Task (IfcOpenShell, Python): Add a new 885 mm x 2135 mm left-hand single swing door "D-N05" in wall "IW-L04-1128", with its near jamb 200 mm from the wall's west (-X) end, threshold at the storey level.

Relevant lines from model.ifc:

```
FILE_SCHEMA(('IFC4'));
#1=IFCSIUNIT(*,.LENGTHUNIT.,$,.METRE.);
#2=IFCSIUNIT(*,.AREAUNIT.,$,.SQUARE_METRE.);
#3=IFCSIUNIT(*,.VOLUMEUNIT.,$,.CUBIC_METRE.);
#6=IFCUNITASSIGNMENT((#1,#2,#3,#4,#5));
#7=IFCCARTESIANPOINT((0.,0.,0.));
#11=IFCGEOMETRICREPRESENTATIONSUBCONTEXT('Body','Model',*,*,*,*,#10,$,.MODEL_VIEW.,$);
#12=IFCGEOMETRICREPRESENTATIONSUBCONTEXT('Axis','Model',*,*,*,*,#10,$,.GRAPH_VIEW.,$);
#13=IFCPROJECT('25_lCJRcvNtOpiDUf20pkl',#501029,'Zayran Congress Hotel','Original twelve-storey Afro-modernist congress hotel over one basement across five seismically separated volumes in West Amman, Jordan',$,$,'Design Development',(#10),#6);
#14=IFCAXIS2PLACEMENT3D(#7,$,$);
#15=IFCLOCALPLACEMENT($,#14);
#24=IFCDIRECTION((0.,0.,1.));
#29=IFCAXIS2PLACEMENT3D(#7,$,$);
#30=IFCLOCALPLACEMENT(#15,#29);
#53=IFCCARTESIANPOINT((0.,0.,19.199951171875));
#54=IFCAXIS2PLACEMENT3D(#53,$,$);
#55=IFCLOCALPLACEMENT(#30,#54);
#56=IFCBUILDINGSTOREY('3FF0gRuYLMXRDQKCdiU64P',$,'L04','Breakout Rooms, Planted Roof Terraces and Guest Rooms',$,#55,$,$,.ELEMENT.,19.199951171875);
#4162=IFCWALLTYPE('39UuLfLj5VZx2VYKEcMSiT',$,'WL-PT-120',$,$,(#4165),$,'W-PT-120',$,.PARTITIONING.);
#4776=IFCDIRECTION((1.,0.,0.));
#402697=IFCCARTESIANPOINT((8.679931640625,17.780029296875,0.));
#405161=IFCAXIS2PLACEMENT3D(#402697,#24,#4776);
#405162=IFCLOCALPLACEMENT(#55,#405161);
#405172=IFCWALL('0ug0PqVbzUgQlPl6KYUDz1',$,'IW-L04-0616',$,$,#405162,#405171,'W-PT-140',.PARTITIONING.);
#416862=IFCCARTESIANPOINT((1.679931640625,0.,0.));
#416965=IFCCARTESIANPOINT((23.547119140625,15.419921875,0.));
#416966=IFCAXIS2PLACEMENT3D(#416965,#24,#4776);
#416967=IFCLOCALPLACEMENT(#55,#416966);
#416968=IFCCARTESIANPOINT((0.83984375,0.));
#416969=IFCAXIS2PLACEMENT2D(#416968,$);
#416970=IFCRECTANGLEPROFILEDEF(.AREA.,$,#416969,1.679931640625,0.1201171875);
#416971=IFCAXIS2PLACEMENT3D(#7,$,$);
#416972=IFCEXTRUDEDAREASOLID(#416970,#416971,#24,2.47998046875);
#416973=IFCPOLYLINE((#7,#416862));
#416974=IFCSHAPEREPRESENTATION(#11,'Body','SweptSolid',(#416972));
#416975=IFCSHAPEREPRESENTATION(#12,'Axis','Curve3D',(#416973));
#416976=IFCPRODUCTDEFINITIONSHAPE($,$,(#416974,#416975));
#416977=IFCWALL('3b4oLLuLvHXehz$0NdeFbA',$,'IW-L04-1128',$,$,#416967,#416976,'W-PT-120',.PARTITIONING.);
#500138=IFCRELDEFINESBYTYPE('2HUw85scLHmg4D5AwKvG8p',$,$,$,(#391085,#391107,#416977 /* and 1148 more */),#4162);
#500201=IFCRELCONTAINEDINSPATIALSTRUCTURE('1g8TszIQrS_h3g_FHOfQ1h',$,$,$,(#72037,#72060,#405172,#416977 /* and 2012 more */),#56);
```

```python
import numpy as np
import ifcopenshell
import ifcopenshell.api.feature
import ifcopenshell.api.geometry
import ifcopenshell.api.root
import ifcopenshell.api.spatial
import ifcopenshell.geom
import ifcopenshell.util.element
import ifcopenshell.util.placement
import ifcopenshell.util.representation
import ifcopenshell.util.shape
import ifcopenshell.util.unit

model = ifcopenshell.open("model.ifc")
unit_scale = ifcopenshell.util.unit.calculate_unit_scale(model)
settings = ifcopenshell.geom.settings()


def volume(element):
    """Net volume in cubic metres, openings subtracted."""
    shape = ifcopenshell.geom.create_shape(settings, element)
    return ifcopenshell.util.shape.get_volume(shape.geometry)


wall = model.by_id(416977)
storey = ifcopenshell.util.element.get_container(wall, ifc_class="IfcBuildingStorey")
context = ifcopenshell.util.representation.get_context(model, "Model", "Body", "MODEL_VIEW")
before = volume(wall)

width, height, from_end, sill = 0.885, 2.135, 0.2, 0.0  # metres

# The wall runs along its own X axis, and the end named is its -X end.
wall_shape = ifcopenshell.geom.create_shape(settings, wall)
x, y, z = ifcopenshell.util.shape.get_vertices(wall_shape.geometry).T
start = x.min() + from_end
face, thickness = float(y.min()), float(y.max() - y.min())
wall_matrix = ifcopenshell.util.placement.get_local_placement(wall.ObjectPlacement)
level = ifcopenshell.util.placement.get_local_placement(storey.ObjectPlacement)[2, 3]


def in_wall(x, y):
    """Placement at x, y metres in the wall's axes, at sill height."""
    matrix = wall_matrix.copy()
    matrix[:, 3] = wall_matrix @ np.array([x / unit_scale, y / unit_scale, 0.0, 1.0])
    matrix[2, 3] = level + sill / unit_scale
    return matrix


# Opening: a box that overshoots both wall faces by 50 mm.
opening = ifcopenshell.api.root.create_entity(model, ifc_class="IfcOpeningElement", predefined_type="OPENING")
box = ifcopenshell.api.geometry.add_wall_representation(
    model, context=context, length=width, height=height, thickness=thickness + 0.1
)
ifcopenshell.api.geometry.assign_representation(model, product=opening, representation=box)
ifcopenshell.api.geometry.edit_object_placement(model, product=opening, matrix=in_wall(start, face - 0.05), is_si=False)
ifcopenshell.api.feature.add_feature(model, feature=opening, element=wall)

door = ifcopenshell.api.root.create_entity(model, ifc_class="IfcDoor", name="D-N05", predefined_type="DOOR")
door.OverallWidth, door.OverallHeight = width / unit_scale, height / unit_scale
door.OperationType = "SINGLE_SWING_LEFT"
body = ifcopenshell.api.geometry.add_door_representation(
    model,
    context=context,
    overall_width=door.OverallWidth,
    overall_height=door.OverallHeight,
    operation_type="SINGLE_SWING_LEFT",
    lining_properties={"LiningDepth": thickness / unit_scale, "ThresholdDepth": thickness / unit_scale},
)
ifcopenshell.api.geometry.assign_representation(model, product=door, representation=body)
ifcopenshell.api.spatial.assign_container(model, products=[door], relating_structure=storey)
ifcopenshell.api.feature.add_filling(model, opening=opening, element=door)

# The lining spans the wall, so the door starts at the wall face.
ifcopenshell.api.geometry.edit_object_placement(model, product=door, matrix=in_wall(start, face), is_si=False)

after = volume(wall)

print(f"wall volume {before:.3f} -> {after:.3f} m3")

model.write("model_edited.ifc")
```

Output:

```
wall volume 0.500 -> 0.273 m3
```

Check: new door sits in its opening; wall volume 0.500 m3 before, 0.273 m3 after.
